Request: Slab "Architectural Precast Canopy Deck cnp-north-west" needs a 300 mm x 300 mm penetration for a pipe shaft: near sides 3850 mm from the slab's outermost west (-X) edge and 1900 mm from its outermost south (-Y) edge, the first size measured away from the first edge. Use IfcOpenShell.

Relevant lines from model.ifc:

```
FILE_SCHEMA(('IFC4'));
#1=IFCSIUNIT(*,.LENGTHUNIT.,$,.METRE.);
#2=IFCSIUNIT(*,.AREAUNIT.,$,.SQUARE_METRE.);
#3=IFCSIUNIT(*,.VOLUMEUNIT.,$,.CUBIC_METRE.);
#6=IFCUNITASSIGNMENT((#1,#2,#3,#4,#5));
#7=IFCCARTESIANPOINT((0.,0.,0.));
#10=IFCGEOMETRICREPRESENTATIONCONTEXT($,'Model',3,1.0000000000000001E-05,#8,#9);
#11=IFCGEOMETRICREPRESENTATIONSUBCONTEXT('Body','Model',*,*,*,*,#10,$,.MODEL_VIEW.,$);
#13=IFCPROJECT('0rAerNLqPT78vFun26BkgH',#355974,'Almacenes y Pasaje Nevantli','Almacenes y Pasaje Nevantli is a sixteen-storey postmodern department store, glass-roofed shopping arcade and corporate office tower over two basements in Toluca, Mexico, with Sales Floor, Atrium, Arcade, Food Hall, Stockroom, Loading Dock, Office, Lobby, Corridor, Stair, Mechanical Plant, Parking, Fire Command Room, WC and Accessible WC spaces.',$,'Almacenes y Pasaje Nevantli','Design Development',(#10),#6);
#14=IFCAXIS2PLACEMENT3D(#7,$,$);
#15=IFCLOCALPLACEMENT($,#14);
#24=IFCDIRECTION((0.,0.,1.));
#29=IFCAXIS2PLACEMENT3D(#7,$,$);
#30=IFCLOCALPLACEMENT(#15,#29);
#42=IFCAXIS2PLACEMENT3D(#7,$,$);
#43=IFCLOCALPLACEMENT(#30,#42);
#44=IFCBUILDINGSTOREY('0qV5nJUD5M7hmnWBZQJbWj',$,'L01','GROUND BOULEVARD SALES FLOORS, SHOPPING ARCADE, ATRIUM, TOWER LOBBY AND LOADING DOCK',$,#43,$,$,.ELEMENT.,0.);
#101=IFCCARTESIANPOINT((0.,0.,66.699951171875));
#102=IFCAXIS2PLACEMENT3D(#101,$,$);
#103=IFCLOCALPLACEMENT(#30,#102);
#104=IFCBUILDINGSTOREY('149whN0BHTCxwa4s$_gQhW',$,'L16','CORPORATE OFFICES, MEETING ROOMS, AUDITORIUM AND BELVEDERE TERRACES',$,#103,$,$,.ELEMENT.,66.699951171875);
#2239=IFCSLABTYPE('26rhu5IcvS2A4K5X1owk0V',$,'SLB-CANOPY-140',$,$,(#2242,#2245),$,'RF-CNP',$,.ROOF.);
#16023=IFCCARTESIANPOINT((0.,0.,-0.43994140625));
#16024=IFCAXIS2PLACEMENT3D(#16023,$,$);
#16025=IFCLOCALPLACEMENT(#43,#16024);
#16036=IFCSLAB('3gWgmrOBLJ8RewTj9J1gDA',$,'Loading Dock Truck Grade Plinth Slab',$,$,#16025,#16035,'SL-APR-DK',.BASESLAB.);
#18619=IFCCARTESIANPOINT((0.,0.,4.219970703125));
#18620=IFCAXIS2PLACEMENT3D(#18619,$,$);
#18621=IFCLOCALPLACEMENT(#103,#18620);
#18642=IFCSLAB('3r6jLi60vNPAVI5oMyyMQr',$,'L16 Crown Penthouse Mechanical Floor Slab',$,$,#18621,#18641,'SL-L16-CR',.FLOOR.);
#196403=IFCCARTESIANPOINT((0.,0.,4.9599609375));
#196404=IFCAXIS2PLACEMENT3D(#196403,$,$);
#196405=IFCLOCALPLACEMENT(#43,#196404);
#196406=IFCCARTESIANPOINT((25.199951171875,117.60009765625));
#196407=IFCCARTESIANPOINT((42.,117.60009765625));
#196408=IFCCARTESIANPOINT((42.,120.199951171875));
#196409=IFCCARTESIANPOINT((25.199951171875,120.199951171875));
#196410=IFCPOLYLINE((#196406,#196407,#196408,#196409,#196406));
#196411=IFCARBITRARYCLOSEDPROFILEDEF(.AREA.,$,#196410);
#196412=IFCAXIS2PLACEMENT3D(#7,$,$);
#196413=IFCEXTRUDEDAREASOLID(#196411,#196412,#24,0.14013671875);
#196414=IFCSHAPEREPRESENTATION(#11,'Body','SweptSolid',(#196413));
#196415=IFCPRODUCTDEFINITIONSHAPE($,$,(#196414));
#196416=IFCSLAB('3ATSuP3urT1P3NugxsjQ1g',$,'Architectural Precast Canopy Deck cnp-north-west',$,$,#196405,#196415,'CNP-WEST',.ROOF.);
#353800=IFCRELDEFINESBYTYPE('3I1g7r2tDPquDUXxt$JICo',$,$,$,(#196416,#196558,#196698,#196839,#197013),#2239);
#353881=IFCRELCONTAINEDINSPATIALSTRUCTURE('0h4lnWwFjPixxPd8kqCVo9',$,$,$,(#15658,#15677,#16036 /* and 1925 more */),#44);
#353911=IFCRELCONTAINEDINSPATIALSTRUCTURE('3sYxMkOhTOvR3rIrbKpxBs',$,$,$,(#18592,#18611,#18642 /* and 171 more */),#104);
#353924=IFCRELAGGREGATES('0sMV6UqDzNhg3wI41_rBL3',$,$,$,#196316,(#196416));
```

```python
import numpy as np
import ifcopenshell
import ifcopenshell.api.feature
import ifcopenshell.api.geometry
import ifcopenshell.api.root
import ifcopenshell.geom
import ifcopenshell.util.placement
import ifcopenshell.util.representation
import ifcopenshell.util.shape
import ifcopenshell.util.unit

model = ifcopenshell.open("model.ifc")
unit_scale = ifcopenshell.util.unit.calculate_unit_scale(model)
settings = ifcopenshell.geom.settings()


def volume(element):
    """Net volume in cubic metres, openings subtracted."""
    shape = ifcopenshell.geom.create_shape(settings, element)
    return ifcopenshell.util.shape.get_volume(shape.geometry)


slab = model.by_guid("3ATSuP3urT1P3NugxsjQ1g")
before = volume(slab)

# Extent in the slab's own axes, in metres. The edges named are its -X and -Y sides.
slab_shape = ifcopenshell.geom.create_shape(settings, slab)
vertices = ifcopenshell.util.shape.get_vertices(slab_shape.geometry)
x_min, y_min, bottom = vertices.min(axis=0)
top = vertices[:, 2].max()

opening = ifcopenshell.api.root.create_entity(model, ifc_class="IfcOpeningElement", name="Pipe shaft opening", predefined_type="OPENING")
context = ifcopenshell.util.representation.get_context(model, "Model", "Body", "MODEL_VIEW")
width, depth = 0.3, 0.3
outline = [(0.0, 0.0), (width, 0.0), (width, depth), (0.0, depth), (0.0, 0.0)]
# Overshoot both faces by 50 mm so the cut is clean.
shape = ifcopenshell.api.geometry.add_slab_representation(
    model, context=context, depth=top - bottom + 0.1, polyline=outline
)
ifcopenshell.api.geometry.assign_representation(model, product=opening, representation=shape)

matrix = ifcopenshell.util.placement.get_local_placement(slab.ObjectPlacement)
matrix[:, 3] = matrix @ np.append(np.array([x_min + 3.85, y_min + 1.9, bottom - 0.05]) / unit_scale, 1.0)
ifcopenshell.api.geometry.edit_object_placement(model, product=opening, matrix=matrix, is_si=False)
ifcopenshell.api.feature.add_feature(model, feature=opening, element=slab)

after = volume(slab)

print(f"slab volume {before:.3f} -> {after:.3f} m3")

model.write("model-out.ifc")
```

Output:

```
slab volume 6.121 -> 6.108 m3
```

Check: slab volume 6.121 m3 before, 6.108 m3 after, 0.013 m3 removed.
